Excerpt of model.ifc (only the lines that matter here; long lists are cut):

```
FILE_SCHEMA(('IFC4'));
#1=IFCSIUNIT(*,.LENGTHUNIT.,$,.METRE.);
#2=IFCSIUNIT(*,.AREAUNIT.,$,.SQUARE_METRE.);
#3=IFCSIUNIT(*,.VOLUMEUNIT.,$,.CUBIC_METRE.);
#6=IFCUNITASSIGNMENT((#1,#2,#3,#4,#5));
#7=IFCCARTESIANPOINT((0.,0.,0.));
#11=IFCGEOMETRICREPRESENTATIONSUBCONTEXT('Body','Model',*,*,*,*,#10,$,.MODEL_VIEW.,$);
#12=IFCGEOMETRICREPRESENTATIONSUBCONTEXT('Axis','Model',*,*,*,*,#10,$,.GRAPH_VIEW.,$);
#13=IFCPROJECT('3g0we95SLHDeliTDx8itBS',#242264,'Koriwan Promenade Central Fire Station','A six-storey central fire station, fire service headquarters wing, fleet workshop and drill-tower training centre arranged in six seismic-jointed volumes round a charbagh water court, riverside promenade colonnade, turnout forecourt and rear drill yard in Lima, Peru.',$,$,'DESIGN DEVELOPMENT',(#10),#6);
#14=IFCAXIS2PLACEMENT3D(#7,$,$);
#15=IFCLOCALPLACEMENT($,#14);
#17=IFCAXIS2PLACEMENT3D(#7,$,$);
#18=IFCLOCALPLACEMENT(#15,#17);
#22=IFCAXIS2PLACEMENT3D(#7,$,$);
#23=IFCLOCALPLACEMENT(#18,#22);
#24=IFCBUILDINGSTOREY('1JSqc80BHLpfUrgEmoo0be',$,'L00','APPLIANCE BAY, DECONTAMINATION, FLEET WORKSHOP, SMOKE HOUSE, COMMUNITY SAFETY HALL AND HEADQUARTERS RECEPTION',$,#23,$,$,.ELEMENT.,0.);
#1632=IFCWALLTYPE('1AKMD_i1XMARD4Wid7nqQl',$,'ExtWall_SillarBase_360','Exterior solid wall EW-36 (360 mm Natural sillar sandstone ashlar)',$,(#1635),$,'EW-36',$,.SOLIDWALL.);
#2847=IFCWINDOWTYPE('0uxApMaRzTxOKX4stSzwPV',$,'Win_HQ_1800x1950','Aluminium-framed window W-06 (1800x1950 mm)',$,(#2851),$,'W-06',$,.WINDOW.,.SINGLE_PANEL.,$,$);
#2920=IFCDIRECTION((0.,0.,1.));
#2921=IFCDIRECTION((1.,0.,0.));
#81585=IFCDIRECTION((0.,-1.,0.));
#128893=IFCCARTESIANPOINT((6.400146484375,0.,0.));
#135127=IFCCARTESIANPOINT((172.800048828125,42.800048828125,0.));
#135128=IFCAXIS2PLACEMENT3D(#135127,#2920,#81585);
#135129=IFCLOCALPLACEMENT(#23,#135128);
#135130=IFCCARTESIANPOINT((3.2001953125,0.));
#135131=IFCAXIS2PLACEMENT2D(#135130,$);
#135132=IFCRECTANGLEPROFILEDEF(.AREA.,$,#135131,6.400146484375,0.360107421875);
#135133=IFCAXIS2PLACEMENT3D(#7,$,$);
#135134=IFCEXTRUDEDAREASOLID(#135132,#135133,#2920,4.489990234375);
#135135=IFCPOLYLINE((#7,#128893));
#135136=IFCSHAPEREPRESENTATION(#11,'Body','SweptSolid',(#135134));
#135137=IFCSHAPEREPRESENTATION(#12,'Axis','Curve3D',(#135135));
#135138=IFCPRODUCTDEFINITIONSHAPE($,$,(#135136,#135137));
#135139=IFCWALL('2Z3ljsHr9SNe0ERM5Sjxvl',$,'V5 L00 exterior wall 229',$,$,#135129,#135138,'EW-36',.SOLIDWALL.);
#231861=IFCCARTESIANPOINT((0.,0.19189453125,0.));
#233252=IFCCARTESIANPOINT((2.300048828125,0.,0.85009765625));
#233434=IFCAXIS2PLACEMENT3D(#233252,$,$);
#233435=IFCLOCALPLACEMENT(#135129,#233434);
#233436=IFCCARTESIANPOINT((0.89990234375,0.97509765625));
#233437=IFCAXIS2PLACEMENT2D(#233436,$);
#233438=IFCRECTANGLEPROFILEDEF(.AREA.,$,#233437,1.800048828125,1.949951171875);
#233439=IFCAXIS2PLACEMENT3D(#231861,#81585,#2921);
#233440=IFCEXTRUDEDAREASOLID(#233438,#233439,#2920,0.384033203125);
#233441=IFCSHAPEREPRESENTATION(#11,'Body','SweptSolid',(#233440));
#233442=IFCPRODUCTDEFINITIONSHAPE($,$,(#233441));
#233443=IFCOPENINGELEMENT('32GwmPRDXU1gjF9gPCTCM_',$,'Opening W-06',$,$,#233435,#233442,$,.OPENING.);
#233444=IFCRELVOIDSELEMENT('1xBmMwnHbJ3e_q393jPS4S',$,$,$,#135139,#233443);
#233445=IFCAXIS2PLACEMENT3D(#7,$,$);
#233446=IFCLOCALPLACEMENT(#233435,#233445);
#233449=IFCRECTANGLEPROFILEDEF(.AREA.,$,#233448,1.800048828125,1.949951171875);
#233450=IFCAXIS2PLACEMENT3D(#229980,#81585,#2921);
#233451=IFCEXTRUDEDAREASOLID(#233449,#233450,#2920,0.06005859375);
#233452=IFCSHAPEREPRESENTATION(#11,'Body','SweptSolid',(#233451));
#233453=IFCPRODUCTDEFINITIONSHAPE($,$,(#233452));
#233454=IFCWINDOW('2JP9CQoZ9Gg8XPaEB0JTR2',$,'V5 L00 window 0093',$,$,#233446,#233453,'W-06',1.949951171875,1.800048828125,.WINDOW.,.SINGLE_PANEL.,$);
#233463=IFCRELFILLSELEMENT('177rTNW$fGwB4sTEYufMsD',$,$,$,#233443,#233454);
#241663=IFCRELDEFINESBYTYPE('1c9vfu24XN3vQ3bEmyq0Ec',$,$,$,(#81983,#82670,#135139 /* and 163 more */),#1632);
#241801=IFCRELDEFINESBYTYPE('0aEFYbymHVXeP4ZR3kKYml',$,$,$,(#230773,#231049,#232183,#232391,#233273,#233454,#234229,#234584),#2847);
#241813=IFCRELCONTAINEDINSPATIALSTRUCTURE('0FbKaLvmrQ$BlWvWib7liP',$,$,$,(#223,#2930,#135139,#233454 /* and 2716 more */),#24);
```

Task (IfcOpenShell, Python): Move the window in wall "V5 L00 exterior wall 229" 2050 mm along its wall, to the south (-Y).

```python
import ifcopenshell
import ifcopenshell.api.geometry
import ifcopenshell.util.placement
import ifcopenshell.util.unit

model = ifcopenshell.open("model.ifc")
unit_scale = ifcopenshell.util.unit.calculate_unit_scale(model)

window = model.by_guid("2JP9CQoZ9Gg8XPaEB0JTR2")
opening = window.FillsVoids[0].RelatingOpeningElement
wall = opening.VoidsElements[0].RelatingBuildingElement

wall_matrix = ifcopenshell.util.placement.get_local_placement(wall.ObjectPlacement)
shift = wall_matrix[:3, 0] * 2.05 / unit_scale
before = ifcopenshell.util.placement.get_local_placement(window.ObjectPlacement)[:3, 3].copy()

# The window is placed relative to its opening, so it follows when the opening moves.
matrix = ifcopenshell.util.placement.get_local_placement(opening.ObjectPlacement)
matrix[:3, 3] += shift
ifcopenshell.api.geometry.edit_object_placement(
    model, product=opening, matrix=matrix, is_si=False, should_transform_children=True
)

after = ifcopenshell.util.placement.get_local_placement(window.ObjectPlacement)[:3, 3]
print("window moved by", (after - before).round(3) + 0.0)

model.write("model_v2.ifc")
```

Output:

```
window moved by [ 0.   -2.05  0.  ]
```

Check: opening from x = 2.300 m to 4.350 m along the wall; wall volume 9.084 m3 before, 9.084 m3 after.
